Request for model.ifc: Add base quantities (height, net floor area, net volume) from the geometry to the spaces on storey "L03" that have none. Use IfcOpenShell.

First a look at what the model holds.

```python
import ifcopenshell
import ifcopenshell.util.element
import ifcopenshell.util.unit

model = ifcopenshell.open("model.ifc")
print(model.schema)
for unit_type in ("LENGTHUNIT", "AREAUNIT", "VOLUMEUNIT"):
    print(unit_type, ifcopenshell.util.unit.calculate_unit_scale(model, unit_type))
storey = next(s for s in model.by_type("IfcBuildingStorey") if s.Name == "L03")
spaces = [e for e in ifcopenshell.util.element.get_decomposition(storey) if e.is_a("IfcSpace")]
for e in sorted(spaces, key=lambda e: e.id()):
    print(e.id(), e.is_a(), e.Name, list(ifcopenshell.util.element.get_psets(e, qtos_only=True)), sep=" | ")
```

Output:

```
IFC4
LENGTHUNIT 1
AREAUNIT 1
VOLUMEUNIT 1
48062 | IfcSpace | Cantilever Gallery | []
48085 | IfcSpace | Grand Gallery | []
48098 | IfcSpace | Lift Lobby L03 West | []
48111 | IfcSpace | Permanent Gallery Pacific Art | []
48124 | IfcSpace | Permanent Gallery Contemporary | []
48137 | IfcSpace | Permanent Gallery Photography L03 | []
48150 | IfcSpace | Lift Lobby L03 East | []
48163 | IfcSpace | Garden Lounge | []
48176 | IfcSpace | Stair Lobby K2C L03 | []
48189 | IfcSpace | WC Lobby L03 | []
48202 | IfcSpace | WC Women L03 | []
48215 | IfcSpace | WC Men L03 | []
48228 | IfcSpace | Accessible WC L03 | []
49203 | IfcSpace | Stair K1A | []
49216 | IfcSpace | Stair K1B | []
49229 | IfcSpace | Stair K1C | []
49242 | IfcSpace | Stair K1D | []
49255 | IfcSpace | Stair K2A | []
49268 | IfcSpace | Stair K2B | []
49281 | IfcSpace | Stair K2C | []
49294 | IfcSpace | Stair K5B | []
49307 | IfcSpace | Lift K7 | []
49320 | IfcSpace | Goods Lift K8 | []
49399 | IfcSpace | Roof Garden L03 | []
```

```python
import ifcopenshell
import ifcopenshell.api.pset
import ifcopenshell.geom
import ifcopenshell.util.element
import ifcopenshell.util.shape
import ifcopenshell.util.unit

model = ifcopenshell.open("model.ifc")
unit_scale = ifcopenshell.util.unit.calculate_unit_scale(model)
area_scale = ifcopenshell.util.unit.calculate_unit_scale(model, "AREAUNIT")
volume_scale = ifcopenshell.util.unit.calculate_unit_scale(model, "VOLUMEUNIT")
settings = ifcopenshell.geom.settings()

storey = next(s for s in model.by_type("IfcBuildingStorey") if s.Name == "L03")
spaces = [e for e in ifcopenshell.util.element.get_decomposition(storey) if e.is_a("IfcSpace")]

for e in sorted(spaces, key=lambda e: e.id()):
    if ifcopenshell.util.element.get_psets(e, qtos_only=True, should_inherit=False):
        continue
    # Geometry comes back in metres, in the element's own axes.
    shape = ifcopenshell.geom.create_shape(settings, e)
    values = {
        "Height": ifcopenshell.util.shape.get_z(shape.geometry) / unit_scale,
        "NetFloorArea": ifcopenshell.util.shape.get_footprint_area(shape.geometry) / area_scale,
        "NetVolume": ifcopenshell.util.shape.get_volume(shape.geometry) / volume_scale,
    }
    qto = ifcopenshell.api.pset.add_qto(model, product=e, name="Qto_SpaceBaseQuantities")
    ifcopenshell.api.pset.edit_qto(model, qto=qto, properties=values)
    print(e.id(), {k: round(v, 3) for k, v in values.items()})

model.write("model_edited.ifc")
```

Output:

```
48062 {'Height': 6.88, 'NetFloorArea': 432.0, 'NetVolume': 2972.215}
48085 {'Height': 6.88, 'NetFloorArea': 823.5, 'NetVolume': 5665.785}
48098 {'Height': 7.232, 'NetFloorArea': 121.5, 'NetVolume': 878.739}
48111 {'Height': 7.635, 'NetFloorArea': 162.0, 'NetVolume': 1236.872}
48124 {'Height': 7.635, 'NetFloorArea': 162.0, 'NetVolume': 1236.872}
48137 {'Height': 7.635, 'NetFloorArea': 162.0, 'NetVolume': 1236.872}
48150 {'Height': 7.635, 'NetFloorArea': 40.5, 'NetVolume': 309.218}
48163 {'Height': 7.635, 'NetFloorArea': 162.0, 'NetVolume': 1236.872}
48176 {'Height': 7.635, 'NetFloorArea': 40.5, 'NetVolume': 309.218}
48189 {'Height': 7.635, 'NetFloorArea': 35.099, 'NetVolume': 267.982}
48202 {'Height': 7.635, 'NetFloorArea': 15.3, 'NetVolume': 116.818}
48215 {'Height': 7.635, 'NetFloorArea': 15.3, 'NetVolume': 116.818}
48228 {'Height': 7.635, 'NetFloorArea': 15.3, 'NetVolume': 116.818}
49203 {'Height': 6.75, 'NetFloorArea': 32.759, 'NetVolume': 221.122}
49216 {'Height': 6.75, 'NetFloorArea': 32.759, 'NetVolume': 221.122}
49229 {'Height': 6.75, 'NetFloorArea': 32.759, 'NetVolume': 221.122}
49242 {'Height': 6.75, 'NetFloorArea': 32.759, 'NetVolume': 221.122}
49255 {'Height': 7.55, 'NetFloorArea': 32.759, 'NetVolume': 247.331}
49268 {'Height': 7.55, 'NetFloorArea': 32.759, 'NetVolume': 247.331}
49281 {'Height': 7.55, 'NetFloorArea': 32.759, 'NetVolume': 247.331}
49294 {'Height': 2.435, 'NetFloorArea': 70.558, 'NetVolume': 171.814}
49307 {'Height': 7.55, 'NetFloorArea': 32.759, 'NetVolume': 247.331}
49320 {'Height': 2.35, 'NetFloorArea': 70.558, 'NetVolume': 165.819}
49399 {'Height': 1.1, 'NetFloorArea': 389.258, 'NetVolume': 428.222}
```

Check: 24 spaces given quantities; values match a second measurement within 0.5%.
